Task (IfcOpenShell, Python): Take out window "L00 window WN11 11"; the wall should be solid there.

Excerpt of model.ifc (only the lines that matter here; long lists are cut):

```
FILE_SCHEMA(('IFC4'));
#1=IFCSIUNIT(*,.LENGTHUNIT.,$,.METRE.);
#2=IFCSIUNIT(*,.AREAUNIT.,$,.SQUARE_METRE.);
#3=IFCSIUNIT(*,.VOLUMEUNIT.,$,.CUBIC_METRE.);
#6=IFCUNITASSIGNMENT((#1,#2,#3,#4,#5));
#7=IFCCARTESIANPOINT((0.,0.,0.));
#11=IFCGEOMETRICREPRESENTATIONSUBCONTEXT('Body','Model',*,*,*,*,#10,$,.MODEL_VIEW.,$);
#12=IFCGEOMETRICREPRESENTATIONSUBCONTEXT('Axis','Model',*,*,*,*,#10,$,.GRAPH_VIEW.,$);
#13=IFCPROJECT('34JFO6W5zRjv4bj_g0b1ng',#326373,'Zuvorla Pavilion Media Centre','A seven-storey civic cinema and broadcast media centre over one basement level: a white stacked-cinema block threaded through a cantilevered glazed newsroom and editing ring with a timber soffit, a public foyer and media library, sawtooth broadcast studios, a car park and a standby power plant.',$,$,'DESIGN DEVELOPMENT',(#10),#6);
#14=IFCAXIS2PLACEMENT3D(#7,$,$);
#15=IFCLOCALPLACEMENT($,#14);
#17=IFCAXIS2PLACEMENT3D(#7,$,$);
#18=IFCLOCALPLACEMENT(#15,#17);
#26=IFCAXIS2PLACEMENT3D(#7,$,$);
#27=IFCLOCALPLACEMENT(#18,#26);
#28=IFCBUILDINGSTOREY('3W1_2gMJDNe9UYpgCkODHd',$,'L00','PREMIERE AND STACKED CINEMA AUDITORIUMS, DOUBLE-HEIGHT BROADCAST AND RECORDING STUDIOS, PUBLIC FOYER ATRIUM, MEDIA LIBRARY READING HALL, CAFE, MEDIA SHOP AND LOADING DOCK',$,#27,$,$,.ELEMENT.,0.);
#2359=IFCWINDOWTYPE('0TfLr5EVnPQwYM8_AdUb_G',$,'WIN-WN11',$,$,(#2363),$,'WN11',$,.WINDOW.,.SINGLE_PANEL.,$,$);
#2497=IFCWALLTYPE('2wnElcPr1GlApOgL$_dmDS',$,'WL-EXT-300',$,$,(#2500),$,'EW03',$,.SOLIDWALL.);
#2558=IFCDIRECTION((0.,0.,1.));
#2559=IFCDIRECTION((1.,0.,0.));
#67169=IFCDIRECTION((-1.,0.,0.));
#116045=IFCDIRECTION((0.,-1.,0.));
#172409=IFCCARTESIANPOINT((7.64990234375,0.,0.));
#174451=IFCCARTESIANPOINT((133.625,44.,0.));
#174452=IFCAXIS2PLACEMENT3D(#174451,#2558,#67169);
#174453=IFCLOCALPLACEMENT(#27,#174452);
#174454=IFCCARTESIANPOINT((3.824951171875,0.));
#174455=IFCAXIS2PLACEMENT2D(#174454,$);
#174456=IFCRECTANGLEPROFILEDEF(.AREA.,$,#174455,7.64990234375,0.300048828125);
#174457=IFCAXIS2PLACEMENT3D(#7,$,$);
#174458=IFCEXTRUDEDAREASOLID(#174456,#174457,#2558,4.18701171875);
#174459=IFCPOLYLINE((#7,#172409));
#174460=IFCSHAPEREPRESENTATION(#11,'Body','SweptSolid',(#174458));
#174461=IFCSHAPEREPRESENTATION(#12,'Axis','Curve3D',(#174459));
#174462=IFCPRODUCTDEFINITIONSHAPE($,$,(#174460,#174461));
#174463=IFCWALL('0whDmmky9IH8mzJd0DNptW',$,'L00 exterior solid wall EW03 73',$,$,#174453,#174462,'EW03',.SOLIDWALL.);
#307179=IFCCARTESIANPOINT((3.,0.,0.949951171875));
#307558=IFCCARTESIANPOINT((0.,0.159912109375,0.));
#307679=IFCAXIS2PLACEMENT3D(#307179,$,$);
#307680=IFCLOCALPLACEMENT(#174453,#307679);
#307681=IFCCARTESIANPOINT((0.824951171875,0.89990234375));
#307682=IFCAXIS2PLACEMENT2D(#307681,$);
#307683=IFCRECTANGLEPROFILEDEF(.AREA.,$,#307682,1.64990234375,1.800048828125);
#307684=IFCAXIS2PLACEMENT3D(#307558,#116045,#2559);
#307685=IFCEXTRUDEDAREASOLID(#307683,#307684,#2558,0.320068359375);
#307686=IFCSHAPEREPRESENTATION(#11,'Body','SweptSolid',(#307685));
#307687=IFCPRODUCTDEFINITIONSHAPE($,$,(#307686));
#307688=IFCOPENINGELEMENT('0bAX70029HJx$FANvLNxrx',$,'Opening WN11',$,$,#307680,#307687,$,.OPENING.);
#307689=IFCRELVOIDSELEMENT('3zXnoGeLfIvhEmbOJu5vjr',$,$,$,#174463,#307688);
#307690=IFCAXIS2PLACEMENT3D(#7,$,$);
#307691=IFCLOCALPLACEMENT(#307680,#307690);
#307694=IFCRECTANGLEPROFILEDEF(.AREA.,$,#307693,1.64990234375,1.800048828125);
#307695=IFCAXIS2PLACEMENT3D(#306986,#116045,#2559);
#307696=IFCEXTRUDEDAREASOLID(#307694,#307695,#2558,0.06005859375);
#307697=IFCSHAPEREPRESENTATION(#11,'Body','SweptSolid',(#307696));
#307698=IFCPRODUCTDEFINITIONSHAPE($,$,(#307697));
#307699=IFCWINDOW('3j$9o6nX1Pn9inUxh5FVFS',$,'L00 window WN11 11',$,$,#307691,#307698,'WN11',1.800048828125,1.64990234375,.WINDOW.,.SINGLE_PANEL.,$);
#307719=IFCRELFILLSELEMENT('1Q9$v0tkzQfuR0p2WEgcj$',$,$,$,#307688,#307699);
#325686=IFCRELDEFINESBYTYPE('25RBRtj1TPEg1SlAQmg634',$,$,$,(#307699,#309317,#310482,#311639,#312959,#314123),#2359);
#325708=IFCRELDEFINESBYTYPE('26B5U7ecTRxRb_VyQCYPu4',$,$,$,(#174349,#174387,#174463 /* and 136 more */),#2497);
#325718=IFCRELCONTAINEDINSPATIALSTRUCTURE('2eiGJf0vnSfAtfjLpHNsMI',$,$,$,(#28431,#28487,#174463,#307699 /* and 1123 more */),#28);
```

```python
import ifcopenshell
import ifcopenshell.api.feature
import ifcopenshell.api.root
import ifcopenshell.geom
import ifcopenshell.util.shape

model = ifcopenshell.open("model.ifc")
settings = ifcopenshell.geom.settings()


def volume(element):
    """Net volume in cubic metres, openings subtracted."""
    shape = ifcopenshell.geom.create_shape(settings, element)
    return ifcopenshell.util.shape.get_volume(shape.geometry)


window = model.by_guid("3j$9o6nX1Pn9inUxh5FVFS")
opening = window.FillsVoids[0].RelatingOpeningElement
wall = opening.VoidsElements[0].RelatingBuildingElement
before = volume(wall)

ifcopenshell.api.root.remove_product(model, product=window)
ifcopenshell.api.feature.remove_feature(model, feature=opening)

after = volume(wall)

print(f"wall volume {before:.3f} -> {after:.3f} m3")

model.write("model_edited.ifc")
```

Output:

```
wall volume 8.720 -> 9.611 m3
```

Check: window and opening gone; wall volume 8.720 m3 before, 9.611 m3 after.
